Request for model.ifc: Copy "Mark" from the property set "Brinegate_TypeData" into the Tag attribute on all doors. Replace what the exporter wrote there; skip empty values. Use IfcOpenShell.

First a look at what the model holds.

```python
import ifcopenshell
import ifcopenshell.util.element

model = ifcopenshell.open("model.ifc")
print(model.schema)
doors = model.by_type("IfcDoor")
print(len(doors), "doors")
for e in doors[:8]:
    source = ifcopenshell.util.element.get_pset(e, "Brinegate_TypeData", "Mark")
    target = e.Tag
    print(e.id(), repr(source), repr(target), sep=" | ")
```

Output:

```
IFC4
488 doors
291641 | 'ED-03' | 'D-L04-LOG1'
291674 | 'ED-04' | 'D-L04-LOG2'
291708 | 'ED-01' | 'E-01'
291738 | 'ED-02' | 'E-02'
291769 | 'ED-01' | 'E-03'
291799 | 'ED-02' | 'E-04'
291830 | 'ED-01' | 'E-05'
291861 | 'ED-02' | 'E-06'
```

```python
import ifcopenshell
import ifcopenshell.util.element

model = ifcopenshell.open("model.ifc")

count = 0
for e in model.by_type("IfcDoor"):
    value = ifcopenshell.util.element.get_pset(e, "Brinegate_TypeData", "Mark")
    current = e.Tag
    if not value or not value.strip() or current == value:
        continue
    e.Tag = value
    count += 1

print(count, "doors updated")

model.write("model_v2.ifc")
```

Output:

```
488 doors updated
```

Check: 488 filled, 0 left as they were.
